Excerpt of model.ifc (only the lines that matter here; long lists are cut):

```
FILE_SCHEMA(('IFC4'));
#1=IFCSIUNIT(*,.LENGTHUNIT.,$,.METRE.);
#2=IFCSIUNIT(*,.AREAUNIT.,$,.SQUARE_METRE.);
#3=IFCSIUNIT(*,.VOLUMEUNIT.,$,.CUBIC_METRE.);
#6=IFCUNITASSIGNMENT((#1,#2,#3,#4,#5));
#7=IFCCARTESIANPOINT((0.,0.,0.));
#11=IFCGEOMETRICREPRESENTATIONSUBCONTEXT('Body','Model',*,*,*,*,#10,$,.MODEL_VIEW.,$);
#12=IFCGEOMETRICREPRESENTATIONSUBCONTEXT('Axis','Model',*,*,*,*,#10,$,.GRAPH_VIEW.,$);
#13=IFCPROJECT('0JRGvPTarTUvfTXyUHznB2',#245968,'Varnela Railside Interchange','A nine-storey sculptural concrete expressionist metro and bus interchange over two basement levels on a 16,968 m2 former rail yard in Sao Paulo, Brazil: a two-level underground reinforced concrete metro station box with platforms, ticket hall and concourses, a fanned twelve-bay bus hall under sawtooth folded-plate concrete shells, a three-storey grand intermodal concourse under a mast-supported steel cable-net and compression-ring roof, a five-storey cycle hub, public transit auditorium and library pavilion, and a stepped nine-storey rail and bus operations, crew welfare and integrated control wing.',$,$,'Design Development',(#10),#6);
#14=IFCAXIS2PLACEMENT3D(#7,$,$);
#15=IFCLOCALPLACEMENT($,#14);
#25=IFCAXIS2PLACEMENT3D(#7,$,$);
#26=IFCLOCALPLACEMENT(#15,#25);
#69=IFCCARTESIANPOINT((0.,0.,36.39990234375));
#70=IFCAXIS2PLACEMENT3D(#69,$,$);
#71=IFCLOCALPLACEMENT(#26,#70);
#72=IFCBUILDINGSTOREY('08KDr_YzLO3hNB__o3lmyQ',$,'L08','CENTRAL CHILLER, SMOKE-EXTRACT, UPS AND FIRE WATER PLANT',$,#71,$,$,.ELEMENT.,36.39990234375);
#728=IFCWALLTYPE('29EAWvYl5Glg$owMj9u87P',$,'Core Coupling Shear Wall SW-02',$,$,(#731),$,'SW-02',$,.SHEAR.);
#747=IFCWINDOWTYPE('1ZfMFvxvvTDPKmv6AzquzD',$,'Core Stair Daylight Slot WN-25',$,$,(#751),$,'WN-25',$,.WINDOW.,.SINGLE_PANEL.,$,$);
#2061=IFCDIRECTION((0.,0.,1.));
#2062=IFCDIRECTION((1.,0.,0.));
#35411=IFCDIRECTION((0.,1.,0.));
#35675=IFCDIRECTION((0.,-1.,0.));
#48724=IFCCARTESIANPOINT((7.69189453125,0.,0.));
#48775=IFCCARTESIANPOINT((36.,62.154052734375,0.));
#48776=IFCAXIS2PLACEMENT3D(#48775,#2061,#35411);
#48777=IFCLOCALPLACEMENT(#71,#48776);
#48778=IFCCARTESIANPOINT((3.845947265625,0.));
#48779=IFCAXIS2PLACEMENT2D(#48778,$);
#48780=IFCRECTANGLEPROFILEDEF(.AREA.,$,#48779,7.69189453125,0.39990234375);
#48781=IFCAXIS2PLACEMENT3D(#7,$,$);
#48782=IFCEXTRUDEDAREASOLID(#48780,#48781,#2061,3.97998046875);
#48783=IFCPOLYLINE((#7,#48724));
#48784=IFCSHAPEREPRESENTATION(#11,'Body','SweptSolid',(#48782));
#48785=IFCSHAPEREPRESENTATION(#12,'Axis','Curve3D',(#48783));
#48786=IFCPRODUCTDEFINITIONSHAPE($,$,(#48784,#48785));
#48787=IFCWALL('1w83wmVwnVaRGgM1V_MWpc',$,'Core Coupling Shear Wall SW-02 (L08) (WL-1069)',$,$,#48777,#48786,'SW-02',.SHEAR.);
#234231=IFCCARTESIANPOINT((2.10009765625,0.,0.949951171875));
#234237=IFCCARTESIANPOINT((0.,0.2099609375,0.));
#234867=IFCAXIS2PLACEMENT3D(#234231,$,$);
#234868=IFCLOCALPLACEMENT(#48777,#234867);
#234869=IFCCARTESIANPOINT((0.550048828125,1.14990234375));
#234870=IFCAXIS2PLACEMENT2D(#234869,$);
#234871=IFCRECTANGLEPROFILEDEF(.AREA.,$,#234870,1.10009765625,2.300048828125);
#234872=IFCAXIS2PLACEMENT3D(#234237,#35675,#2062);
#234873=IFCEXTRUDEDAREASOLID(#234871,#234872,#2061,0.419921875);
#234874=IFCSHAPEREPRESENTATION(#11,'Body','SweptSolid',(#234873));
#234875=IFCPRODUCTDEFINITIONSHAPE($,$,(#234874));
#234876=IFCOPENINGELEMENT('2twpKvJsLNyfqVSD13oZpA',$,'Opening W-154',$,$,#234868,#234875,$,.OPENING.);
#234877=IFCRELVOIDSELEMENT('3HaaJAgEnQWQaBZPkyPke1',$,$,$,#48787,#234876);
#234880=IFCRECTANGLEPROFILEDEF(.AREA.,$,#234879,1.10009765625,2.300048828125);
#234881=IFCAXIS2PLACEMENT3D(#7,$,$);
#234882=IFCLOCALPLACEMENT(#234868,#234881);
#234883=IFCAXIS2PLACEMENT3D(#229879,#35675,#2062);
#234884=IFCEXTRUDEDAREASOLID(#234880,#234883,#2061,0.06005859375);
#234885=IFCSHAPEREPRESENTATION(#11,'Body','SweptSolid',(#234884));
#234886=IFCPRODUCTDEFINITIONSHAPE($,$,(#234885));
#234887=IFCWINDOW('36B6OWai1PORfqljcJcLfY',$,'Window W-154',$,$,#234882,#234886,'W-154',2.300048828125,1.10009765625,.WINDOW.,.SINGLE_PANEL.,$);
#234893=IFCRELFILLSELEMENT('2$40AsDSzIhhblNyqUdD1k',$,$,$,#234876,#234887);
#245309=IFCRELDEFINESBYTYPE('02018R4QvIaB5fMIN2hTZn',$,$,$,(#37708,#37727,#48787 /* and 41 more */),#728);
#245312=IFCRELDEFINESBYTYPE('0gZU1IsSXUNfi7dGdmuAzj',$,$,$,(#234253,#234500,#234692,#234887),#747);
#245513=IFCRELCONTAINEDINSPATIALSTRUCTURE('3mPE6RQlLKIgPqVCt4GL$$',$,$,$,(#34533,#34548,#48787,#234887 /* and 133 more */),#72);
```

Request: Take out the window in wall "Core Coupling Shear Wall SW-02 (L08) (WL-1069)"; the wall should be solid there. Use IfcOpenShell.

```python
import ifcopenshell
import ifcopenshell.api.feature
import ifcopenshell.api.root
import ifcopenshell.geom
import ifcopenshell.util.shape

model = ifcopenshell.open("model.ifc")
settings = ifcopenshell.geom.settings()


def volume(element):
    """Net volume in cubic metres, openings subtracted."""
    shape = ifcopenshell.geom.create_shape(settings, element)
    return ifcopenshell.util.shape.get_volume(shape.geometry)


window = model.by_guid("36B6OWai1PORfqljcJcLfY")
opening = window.FillsVoids[0].RelatingOpeningElement
wall = opening.VoidsElements[0].RelatingBuildingElement
before = volume(wall)

ifcopenshell.api.root.remove_product(model, product=window)
ifcopenshell.api.feature.remove_feature(model, feature=opening)

after = volume(wall)

print(f"wall volume {before:.3f} -> {after:.3f} m3")

model.write("model_updated.ifc")
```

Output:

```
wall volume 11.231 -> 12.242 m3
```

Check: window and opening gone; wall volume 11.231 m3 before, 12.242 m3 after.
